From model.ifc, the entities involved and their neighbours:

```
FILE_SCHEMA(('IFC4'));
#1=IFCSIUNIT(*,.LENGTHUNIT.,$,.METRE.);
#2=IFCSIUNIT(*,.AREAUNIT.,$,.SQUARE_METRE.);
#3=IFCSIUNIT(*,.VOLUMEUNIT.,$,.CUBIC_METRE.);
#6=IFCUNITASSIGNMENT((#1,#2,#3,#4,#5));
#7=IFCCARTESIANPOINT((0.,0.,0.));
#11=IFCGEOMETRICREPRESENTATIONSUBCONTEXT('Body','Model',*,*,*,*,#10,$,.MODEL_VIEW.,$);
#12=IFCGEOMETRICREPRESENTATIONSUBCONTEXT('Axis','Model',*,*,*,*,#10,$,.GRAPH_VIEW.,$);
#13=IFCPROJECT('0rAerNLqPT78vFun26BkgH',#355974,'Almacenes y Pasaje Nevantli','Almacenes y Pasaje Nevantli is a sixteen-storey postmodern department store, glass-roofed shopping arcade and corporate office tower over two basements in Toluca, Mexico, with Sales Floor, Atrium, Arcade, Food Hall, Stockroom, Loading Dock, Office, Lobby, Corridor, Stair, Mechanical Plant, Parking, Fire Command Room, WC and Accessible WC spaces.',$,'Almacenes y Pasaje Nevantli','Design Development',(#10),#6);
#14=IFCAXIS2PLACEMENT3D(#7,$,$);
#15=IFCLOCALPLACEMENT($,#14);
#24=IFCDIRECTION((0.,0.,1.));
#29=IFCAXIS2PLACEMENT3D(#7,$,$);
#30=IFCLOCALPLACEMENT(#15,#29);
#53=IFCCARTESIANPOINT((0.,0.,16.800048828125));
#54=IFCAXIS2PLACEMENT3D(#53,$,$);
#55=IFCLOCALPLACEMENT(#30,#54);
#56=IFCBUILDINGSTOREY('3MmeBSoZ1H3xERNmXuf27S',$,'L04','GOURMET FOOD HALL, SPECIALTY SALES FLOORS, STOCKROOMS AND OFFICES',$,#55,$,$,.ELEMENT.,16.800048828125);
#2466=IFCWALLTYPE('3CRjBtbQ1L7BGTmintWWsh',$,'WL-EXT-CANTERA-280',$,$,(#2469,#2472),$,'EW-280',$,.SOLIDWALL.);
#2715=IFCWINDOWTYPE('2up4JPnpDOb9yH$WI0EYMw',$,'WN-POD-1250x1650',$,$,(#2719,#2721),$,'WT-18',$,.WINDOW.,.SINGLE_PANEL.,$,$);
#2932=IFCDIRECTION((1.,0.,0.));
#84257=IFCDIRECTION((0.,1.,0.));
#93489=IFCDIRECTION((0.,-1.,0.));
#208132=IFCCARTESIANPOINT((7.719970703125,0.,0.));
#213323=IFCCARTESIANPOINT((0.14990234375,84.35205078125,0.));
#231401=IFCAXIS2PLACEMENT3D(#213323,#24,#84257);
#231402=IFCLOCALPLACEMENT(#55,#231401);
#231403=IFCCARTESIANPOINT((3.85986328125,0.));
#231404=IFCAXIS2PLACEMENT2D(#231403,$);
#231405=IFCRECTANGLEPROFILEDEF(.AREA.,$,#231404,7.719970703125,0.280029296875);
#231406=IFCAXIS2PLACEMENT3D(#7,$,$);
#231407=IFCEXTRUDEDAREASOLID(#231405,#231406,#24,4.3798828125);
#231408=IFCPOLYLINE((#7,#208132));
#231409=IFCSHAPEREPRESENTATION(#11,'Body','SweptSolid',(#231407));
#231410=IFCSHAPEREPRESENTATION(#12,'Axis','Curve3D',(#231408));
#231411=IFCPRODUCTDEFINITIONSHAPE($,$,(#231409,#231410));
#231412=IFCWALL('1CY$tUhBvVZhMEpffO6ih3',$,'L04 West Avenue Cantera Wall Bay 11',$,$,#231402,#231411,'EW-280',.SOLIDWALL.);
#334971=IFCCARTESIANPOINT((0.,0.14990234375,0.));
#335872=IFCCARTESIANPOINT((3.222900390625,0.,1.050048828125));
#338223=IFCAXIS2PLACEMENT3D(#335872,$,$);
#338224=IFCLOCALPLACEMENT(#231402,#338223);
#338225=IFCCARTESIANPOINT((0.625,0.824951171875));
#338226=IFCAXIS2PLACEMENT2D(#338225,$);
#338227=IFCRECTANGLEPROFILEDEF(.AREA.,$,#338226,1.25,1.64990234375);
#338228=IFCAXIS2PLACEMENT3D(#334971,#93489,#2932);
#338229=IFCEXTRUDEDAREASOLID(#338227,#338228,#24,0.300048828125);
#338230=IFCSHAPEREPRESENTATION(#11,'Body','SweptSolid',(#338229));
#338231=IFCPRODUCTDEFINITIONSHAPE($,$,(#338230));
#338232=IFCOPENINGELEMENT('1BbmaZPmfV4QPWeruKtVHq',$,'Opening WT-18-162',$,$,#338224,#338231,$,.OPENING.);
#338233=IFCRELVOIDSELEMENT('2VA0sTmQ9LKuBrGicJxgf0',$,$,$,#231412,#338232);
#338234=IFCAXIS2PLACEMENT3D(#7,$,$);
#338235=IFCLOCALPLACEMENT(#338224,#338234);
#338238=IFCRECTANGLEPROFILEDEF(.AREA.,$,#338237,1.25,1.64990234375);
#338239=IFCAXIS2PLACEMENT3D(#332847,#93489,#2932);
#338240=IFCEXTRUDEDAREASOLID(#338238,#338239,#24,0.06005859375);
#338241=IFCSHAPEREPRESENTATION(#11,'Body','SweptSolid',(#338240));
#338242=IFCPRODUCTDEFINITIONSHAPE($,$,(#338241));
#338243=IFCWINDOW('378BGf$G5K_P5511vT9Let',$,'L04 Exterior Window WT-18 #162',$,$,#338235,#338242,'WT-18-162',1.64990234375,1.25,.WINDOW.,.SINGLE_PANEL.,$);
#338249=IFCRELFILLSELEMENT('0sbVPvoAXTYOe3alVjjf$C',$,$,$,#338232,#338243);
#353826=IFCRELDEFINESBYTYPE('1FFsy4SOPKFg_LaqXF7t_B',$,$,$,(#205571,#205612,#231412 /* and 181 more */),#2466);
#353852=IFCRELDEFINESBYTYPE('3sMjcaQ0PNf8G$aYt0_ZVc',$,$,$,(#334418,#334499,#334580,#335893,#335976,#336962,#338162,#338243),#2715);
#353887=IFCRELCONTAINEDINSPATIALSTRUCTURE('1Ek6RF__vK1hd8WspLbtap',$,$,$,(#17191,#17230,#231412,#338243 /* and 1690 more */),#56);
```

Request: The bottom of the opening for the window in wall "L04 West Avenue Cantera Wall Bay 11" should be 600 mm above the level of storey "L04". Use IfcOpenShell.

```python
import numpy as np
import ifcopenshell
import ifcopenshell.api.geometry
import ifcopenshell.geom
import ifcopenshell.util.element
import ifcopenshell.util.placement
import ifcopenshell.util.shape
import ifcopenshell.util.unit

model = ifcopenshell.open("model.ifc")
unit_scale = ifcopenshell.util.unit.calculate_unit_scale(model)

window = model.by_id(338243)
opening = window.FillsVoids[0].RelatingOpeningElement
storey = ifcopenshell.util.element.get_container(window, ifc_class="IfcBuildingStorey")
level = ifcopenshell.util.placement.get_local_placement(storey.ObjectPlacement)[2, 3]

# The opening's origin need not be at the sill, so measure its lowest point.
shape = ifcopenshell.geom.create_shape(ifcopenshell.geom.settings(), opening)
bottom = ifcopenshell.util.shape.get_shape_bottom_elevation(shape, shape.geometry) / unit_scale
dz = level + 0.6 / unit_scale - bottom

shift = np.array([0.0, 0.0, dz])
# The window is placed relative to its opening, so it follows when the opening moves.
matrix = ifcopenshell.util.placement.get_local_placement(opening.ObjectPlacement)
matrix[:3, 3] += shift
ifcopenshell.api.geometry.edit_object_placement(
    model, product=opening, matrix=matrix, is_si=False, should_transform_children=True
)

print(f"moved by {dz * unit_scale:+.3f} m")

model.write("model_edited.ifc")
```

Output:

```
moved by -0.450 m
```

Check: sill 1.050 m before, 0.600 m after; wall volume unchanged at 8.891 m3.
